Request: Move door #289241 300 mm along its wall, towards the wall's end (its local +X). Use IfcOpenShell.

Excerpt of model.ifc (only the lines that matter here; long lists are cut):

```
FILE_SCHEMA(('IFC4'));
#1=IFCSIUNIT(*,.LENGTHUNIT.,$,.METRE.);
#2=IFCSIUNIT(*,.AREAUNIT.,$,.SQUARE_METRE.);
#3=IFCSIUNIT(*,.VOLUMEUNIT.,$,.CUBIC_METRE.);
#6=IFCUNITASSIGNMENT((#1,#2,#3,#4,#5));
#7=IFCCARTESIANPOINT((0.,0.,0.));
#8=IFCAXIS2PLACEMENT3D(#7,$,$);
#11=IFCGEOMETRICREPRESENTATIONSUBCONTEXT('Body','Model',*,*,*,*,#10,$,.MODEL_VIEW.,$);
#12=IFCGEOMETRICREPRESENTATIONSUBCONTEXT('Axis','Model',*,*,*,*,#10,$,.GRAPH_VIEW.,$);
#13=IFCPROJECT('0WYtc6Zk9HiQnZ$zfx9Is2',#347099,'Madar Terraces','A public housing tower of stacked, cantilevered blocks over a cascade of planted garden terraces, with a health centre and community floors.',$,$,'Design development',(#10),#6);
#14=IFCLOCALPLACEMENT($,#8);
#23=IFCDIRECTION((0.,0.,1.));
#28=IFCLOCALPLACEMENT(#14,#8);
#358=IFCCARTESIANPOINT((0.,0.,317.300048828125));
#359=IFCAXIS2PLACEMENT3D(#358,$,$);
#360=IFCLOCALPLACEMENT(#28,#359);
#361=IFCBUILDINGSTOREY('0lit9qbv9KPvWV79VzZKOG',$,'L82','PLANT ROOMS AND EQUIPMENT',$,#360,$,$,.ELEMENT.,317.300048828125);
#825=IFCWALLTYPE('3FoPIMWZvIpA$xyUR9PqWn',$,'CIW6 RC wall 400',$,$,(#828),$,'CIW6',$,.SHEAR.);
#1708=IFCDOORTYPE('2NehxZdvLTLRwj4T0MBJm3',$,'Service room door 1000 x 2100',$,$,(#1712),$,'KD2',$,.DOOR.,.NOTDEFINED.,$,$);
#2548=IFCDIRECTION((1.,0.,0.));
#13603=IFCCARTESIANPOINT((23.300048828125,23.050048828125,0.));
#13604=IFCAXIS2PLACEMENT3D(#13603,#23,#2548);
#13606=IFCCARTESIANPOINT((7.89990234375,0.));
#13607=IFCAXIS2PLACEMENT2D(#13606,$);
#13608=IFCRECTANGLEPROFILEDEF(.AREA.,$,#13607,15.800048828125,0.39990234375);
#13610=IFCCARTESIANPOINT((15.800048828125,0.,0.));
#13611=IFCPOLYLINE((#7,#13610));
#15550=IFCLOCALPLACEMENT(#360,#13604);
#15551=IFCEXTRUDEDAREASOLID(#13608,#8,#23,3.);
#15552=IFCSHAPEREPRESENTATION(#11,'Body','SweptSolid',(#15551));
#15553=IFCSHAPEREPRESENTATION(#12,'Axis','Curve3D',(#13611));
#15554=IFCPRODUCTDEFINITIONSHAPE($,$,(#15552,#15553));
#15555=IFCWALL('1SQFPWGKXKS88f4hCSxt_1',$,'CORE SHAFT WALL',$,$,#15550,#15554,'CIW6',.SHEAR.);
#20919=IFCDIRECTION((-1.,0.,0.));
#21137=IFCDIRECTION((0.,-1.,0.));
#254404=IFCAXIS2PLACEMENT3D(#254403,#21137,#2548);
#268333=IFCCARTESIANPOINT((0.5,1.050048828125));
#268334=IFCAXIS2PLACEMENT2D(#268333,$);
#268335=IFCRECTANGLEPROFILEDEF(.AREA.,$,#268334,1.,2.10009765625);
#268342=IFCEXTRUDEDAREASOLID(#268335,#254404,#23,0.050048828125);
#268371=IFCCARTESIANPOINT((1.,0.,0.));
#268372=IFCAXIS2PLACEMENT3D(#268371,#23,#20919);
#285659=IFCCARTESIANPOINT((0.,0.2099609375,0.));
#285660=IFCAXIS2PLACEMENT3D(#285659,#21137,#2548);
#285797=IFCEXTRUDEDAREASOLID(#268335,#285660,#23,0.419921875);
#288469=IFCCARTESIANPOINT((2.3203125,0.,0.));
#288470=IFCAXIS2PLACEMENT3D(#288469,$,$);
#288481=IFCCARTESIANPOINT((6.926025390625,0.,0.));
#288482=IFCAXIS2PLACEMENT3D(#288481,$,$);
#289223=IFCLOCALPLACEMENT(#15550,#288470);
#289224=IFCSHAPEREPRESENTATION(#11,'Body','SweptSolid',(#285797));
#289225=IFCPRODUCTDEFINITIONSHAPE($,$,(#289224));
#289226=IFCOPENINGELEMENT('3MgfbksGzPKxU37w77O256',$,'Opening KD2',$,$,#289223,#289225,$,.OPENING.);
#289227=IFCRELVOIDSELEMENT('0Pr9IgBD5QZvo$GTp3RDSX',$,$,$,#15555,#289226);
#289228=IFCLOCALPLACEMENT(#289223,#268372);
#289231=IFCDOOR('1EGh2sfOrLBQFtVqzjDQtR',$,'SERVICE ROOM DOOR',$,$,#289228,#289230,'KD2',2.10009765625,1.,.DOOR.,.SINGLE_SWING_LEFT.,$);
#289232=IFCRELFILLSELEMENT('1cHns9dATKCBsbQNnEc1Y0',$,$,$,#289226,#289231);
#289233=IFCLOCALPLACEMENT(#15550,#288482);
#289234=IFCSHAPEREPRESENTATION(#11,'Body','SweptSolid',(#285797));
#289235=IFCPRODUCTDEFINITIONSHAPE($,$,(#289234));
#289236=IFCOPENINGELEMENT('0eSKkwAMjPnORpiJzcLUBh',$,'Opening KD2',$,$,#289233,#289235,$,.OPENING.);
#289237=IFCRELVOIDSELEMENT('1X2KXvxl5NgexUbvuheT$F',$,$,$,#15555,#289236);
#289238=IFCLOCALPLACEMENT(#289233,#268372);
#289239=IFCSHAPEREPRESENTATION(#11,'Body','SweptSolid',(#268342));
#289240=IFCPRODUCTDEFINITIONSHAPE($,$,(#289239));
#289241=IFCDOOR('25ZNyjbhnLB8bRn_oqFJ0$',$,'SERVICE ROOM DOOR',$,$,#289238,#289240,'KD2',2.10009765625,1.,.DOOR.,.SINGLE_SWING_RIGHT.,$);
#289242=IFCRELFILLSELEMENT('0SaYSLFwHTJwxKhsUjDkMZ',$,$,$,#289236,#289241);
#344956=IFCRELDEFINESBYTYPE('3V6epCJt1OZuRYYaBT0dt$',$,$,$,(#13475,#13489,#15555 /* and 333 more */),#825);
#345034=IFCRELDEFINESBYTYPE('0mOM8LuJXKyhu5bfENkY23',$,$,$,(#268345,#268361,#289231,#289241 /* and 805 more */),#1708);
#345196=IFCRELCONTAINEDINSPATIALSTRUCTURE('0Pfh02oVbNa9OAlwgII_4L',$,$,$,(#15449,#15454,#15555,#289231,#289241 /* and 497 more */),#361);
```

```python
import ifcopenshell
import ifcopenshell.api.geometry
import ifcopenshell.util.placement

model = ifcopenshell.open("model.ifc")

door = model.by_guid("25ZNyjbhnLB8bRn_oqFJ0$")
opening = door.FillsVoids[0].RelatingOpeningElement
wall = opening.VoidsElements[0].RelatingBuildingElement

wall_matrix = ifcopenshell.util.placement.get_local_placement(wall.ObjectPlacement)
shift = wall_matrix[:3, 0] * 0.3
before = ifcopenshell.util.placement.get_local_placement(door.ObjectPlacement)[:3, 3].copy()

# The door is placed relative to its opening, so it follows when the opening moves.
matrix = ifcopenshell.util.placement.get_local_placement(opening.ObjectPlacement)
matrix[:3, 3] += shift
ifcopenshell.api.geometry.edit_object_placement(
    model, product=opening, matrix=matrix, is_si=False, should_transform_children=True
)

after = ifcopenshell.util.placement.get_local_placement(door.ObjectPlacement)[:3, 3]
print("door moved by", (after - before).round(3) + 0.0)

model.write("model_edited.ifc")
```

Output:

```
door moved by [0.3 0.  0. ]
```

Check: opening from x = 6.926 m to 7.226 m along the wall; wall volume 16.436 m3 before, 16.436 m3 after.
